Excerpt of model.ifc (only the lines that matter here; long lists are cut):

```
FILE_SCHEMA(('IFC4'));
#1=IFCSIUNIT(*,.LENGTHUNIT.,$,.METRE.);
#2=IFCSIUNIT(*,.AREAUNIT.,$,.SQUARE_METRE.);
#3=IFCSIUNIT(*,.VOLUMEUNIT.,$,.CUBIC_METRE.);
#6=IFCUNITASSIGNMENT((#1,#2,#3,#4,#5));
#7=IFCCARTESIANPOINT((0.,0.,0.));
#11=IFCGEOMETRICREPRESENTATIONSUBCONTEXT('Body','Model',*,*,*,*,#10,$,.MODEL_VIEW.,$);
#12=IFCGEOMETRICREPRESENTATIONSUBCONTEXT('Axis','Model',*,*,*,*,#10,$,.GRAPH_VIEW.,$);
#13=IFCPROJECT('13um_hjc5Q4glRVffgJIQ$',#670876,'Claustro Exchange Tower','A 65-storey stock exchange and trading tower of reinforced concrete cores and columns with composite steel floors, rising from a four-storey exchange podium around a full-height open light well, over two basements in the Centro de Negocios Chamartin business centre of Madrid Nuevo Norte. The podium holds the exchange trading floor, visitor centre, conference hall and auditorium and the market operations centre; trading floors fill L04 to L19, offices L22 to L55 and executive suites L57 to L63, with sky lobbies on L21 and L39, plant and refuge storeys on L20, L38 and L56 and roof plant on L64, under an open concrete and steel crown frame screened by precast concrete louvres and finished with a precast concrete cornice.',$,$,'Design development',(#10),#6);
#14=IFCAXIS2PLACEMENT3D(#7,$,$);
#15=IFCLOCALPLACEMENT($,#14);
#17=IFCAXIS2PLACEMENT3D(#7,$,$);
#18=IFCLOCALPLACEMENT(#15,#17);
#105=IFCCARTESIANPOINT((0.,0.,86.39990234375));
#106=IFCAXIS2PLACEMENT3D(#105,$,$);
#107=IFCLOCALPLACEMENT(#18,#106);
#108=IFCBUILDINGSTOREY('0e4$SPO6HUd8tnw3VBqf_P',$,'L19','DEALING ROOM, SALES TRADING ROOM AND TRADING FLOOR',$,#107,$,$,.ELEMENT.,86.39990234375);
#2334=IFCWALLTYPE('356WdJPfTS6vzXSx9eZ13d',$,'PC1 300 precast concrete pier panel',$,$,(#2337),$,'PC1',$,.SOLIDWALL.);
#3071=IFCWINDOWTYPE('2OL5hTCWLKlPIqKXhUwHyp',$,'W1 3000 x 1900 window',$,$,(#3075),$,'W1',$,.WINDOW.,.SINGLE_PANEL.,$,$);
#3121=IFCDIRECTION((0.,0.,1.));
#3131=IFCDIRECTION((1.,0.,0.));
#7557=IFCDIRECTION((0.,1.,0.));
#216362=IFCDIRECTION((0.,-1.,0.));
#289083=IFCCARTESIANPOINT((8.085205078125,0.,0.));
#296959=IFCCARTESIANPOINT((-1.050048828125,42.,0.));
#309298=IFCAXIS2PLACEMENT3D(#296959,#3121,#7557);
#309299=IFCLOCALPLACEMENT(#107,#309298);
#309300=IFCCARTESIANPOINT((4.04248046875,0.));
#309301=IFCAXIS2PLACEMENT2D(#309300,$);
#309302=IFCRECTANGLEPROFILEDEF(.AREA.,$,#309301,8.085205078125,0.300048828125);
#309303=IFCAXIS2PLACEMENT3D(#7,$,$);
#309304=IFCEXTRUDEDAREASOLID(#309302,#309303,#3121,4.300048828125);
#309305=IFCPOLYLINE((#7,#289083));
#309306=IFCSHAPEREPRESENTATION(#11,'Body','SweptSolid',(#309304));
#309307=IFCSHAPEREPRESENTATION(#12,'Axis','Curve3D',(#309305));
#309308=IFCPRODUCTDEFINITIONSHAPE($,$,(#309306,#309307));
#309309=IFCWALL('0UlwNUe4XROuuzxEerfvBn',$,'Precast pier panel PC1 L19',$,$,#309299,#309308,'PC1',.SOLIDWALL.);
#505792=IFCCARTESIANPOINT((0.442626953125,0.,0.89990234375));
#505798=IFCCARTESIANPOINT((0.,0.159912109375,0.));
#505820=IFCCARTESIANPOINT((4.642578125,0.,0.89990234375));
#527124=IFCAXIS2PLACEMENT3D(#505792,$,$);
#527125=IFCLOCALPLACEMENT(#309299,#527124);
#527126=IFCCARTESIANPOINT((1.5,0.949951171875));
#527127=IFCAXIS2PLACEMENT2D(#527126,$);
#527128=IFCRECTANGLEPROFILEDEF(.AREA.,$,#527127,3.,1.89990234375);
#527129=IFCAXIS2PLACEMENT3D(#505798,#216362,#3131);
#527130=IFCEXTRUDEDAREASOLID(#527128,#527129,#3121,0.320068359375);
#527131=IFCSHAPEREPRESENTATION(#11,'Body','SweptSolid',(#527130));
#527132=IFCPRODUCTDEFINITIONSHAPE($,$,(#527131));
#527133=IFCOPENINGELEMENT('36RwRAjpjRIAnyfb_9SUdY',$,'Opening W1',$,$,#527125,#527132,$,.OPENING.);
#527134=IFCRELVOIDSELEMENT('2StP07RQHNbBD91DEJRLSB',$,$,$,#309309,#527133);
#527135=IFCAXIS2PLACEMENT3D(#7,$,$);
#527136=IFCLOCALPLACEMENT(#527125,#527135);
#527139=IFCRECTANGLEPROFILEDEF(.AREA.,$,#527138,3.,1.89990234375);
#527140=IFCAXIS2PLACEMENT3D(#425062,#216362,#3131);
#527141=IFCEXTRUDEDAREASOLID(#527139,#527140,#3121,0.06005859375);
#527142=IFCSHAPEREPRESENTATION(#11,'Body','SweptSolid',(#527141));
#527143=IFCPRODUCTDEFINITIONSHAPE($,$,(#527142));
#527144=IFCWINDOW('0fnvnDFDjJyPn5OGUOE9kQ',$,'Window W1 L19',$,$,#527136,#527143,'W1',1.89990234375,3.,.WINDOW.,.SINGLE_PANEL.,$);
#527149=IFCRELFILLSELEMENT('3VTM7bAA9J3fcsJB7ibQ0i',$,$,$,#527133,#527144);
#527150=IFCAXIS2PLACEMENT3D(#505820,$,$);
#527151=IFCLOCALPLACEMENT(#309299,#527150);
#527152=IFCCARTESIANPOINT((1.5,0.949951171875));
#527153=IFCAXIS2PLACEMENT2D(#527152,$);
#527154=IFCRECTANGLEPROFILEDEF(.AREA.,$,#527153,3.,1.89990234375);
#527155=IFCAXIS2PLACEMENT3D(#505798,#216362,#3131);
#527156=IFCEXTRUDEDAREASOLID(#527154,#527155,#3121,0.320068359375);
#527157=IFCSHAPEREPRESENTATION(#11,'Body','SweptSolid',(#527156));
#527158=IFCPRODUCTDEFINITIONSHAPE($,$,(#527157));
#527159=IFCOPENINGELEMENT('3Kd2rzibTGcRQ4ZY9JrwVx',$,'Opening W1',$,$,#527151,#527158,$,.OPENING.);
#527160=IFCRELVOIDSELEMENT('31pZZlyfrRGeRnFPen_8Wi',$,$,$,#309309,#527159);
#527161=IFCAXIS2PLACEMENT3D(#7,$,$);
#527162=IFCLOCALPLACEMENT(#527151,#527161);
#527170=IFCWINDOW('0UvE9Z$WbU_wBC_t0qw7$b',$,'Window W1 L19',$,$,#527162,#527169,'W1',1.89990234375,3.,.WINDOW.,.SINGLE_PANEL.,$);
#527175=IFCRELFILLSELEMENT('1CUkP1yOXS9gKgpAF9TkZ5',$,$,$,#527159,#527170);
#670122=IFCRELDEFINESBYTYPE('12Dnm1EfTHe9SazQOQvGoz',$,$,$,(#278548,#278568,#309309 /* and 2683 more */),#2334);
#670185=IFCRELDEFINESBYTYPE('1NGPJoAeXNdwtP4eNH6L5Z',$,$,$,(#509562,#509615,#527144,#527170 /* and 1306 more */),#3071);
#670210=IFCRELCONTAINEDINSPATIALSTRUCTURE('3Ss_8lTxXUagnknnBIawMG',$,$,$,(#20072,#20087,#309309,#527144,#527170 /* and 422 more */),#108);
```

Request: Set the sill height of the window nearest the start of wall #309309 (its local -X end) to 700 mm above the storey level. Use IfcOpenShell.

```python
import numpy as np
import ifcopenshell
import ifcopenshell.api.geometry
import ifcopenshell.geom
import ifcopenshell.util.element
import ifcopenshell.util.placement
import ifcopenshell.util.shape
import ifcopenshell.util.unit

model = ifcopenshell.open("model.ifc")
unit_scale = ifcopenshell.util.unit.calculate_unit_scale(model)

window = model.by_guid("0fnvnDFDjJyPn5OGUOE9kQ")
opening = window.FillsVoids[0].RelatingOpeningElement
storey = ifcopenshell.util.element.get_container(window, ifc_class="IfcBuildingStorey")
level = ifcopenshell.util.placement.get_local_placement(storey.ObjectPlacement)[2, 3]

# The opening's origin need not be at the sill, so measure its lowest point.
shape = ifcopenshell.geom.create_shape(ifcopenshell.geom.settings(), opening)
bottom = ifcopenshell.util.shape.get_shape_bottom_elevation(shape, shape.geometry) / unit_scale
dz = level + 0.7 / unit_scale - bottom

shift = np.array([0.0, 0.0, dz])
# The window is placed relative to its opening, so it follows when the opening moves.
matrix = ifcopenshell.util.placement.get_local_placement(opening.ObjectPlacement)
matrix[:3, 3] += shift
ifcopenshell.api.geometry.edit_object_placement(
    model, product=opening, matrix=matrix, is_si=False, should_transform_children=True
)

print(f"moved by {dz * unit_scale:+.3f} m")

model.write("model_edited.ifc")
```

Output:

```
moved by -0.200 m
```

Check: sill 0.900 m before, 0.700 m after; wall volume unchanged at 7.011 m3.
